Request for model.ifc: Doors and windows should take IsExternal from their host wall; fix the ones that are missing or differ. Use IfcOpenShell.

First a look at what the model holds.

```python
import ifcopenshell
import ifcopenshell.util.element

model = ifcopenshell.open("model.ifc")
print(model.schema)
seen = {}
for e in model.by_type("IfcDoor") + model.by_type("IfcWindow"):
    if not e.FillsVoids:
        continue
    host = e.FillsVoids[0].RelatingOpeningElement.VoidsElements[0].RelatingBuildingElement
    own = ifcopenshell.util.element.get_pset(e, f"Pset_{e.is_a()[3:].removesuffix('StandardCase')}Common", "IsExternal")
    wall = ifcopenshell.util.element.get_pset(host, "Pset_WallCommon", "IsExternal")
    seen[e.is_a(), own, wall] = seen.get((e.is_a(), own, wall), 0) + 1
for (cls, own, wall), count in sorted(seen.items(), key=str):
    print(count, cls, "IsExternal:", own, "| host wall:", wall)
```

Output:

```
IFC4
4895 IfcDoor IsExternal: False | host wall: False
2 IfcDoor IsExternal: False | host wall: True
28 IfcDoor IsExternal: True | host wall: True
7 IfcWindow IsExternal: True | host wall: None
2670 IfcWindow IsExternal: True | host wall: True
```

```python
import ifcopenshell
import ifcopenshell.api.pset
import ifcopenshell.util.element

model = ifcopenshell.open("model.ifc")

count = 0
for ifc_class, pset_name in (("IfcDoor", "Pset_DoorCommon"), ("IfcWindow", "Pset_WindowCommon")):
    for e in model.by_type(ifc_class):
        if not e.FillsVoids:
            continue
        host = e.FillsVoids[0].RelatingOpeningElement.VoidsElements[0].RelatingBuildingElement
        external = ifcopenshell.util.element.get_pset(host, "Pset_WallCommon", "IsExternal")
        if external is None or ifcopenshell.util.element.get_pset(e, pset_name, "IsExternal") == external:
            continue
        found = ifcopenshell.util.element.get_pset(e, pset_name, should_inherit=False)
        if found:
            pset = model.by_id(found["id"])
            if len(ifcopenshell.util.element.get_elements_by_pset(pset)) > 1:
                pset = ifcopenshell.api.pset.unshare_pset(model, products=[e], pset=pset)[0]
        else:
            pset = ifcopenshell.api.pset.add_pset(model, product=e, name=pset_name)
        ifcopenshell.api.pset.edit_pset(model, pset=pset, properties={"IsExternal": external})
        count += 1

print(count, "updated")

model.write("model_updated.ifc")
```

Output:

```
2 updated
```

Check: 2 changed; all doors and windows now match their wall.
